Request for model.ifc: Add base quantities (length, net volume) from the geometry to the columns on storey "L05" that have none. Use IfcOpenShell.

First a look at what the model holds.

```python
import ifcopenshell
import ifcopenshell.util.element
import ifcopenshell.util.unit

model = ifcopenshell.open("model.ifc")
print(model.schema)
for unit_type in ("LENGTHUNIT", "AREAUNIT", "VOLUMEUNIT"):
    print(unit_type, ifcopenshell.util.unit.calculate_unit_scale(model, unit_type))
storey = next(s for s in model.by_type("IfcBuildingStorey") if s.Name == "L05")
columns = [e for e in ifcopenshell.util.element.get_decomposition(storey) if e.is_a("IfcColumn")]
for e in sorted(columns, key=lambda e: e.id()):
    print(e.id(), e.is_a(), e.Name, list(ifcopenshell.util.element.get_psets(e, qtos_only=True)), sep=" | ")
```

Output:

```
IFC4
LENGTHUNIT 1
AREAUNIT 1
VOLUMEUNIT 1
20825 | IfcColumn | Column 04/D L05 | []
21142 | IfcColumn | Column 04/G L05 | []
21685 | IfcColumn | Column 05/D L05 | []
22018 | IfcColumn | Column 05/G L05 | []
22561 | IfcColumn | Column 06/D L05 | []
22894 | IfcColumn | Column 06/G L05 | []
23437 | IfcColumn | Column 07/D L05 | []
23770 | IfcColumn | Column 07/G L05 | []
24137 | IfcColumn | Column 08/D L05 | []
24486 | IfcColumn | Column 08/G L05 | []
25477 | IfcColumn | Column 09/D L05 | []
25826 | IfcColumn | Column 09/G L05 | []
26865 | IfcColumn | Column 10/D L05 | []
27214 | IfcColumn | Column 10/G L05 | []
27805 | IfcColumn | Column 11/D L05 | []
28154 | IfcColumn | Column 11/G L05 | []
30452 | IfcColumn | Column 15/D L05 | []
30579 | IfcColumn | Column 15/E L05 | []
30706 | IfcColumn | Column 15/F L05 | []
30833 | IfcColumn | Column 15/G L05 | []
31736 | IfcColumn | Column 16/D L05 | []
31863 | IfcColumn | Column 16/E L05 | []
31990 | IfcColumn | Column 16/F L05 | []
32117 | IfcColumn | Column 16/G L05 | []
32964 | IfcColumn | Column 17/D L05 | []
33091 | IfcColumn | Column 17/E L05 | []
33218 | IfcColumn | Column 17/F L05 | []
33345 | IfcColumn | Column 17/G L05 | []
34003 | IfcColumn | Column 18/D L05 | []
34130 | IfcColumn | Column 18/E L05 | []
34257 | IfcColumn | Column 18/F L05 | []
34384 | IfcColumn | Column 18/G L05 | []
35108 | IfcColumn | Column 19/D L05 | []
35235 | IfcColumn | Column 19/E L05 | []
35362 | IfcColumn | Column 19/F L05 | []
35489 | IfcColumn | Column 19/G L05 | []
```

```python
import ifcopenshell
import ifcopenshell.api.pset
import ifcopenshell.geom
import ifcopenshell.util.element
import ifcopenshell.util.shape
import ifcopenshell.util.unit

model = ifcopenshell.open("model.ifc")
unit_scale = ifcopenshell.util.unit.calculate_unit_scale(model)
volume_scale = ifcopenshell.util.unit.calculate_unit_scale(model, "VOLUMEUNIT")
settings = ifcopenshell.geom.settings()

storey = next(s for s in model.by_type("IfcBuildingStorey") if s.Name == "L05")
columns = [e for e in ifcopenshell.util.element.get_decomposition(storey) if e.is_a("IfcColumn")]

for e in sorted(columns, key=lambda e: e.id()):
    if ifcopenshell.util.element.get_psets(e, qtos_only=True, should_inherit=False):
        continue
    # Geometry comes back in metres, in the element's own axes.
    shape = ifcopenshell.geom.create_shape(settings, e)
    values = {
        "Length": ifcopenshell.util.shape.get_z(shape.geometry) / unit_scale,
        "NetVolume": ifcopenshell.util.shape.get_volume(shape.geometry) / volume_scale,
    }
    qto = ifcopenshell.api.pset.add_qto(model, product=e, name="Qto_ColumnBaseQuantities")
    ifcopenshell.api.pset.edit_qto(model, qto=qto, properties=values)
    print(e.id(), {k: round(v, 3) for k, v in values.items()})

model.write("model_edited.ifc")
```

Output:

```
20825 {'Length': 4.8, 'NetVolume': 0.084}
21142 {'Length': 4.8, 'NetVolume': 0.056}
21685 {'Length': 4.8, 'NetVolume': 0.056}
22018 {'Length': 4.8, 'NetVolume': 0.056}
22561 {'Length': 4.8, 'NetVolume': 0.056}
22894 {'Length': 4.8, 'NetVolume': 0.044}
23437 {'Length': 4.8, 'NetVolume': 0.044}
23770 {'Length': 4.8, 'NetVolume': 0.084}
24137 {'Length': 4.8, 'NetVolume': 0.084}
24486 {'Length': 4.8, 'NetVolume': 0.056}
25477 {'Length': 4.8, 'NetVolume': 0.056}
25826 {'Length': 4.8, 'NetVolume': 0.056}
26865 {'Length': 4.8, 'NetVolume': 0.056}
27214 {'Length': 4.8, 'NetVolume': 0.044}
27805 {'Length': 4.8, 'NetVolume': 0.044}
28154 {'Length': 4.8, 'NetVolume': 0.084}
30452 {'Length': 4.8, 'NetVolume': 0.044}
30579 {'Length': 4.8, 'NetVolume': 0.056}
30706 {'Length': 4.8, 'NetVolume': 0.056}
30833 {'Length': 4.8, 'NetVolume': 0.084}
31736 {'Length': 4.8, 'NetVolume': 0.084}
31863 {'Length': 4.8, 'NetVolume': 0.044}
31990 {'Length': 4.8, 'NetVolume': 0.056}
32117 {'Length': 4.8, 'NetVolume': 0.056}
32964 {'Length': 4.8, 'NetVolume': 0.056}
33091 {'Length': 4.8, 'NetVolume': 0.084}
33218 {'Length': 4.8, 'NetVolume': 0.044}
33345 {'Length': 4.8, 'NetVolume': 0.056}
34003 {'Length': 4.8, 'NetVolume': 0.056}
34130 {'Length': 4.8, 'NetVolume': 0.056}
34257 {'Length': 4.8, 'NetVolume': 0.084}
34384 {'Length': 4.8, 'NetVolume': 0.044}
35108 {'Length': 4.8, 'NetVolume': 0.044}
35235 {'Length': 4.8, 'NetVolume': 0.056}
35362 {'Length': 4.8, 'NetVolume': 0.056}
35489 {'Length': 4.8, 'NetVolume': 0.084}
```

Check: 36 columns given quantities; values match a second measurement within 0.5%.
